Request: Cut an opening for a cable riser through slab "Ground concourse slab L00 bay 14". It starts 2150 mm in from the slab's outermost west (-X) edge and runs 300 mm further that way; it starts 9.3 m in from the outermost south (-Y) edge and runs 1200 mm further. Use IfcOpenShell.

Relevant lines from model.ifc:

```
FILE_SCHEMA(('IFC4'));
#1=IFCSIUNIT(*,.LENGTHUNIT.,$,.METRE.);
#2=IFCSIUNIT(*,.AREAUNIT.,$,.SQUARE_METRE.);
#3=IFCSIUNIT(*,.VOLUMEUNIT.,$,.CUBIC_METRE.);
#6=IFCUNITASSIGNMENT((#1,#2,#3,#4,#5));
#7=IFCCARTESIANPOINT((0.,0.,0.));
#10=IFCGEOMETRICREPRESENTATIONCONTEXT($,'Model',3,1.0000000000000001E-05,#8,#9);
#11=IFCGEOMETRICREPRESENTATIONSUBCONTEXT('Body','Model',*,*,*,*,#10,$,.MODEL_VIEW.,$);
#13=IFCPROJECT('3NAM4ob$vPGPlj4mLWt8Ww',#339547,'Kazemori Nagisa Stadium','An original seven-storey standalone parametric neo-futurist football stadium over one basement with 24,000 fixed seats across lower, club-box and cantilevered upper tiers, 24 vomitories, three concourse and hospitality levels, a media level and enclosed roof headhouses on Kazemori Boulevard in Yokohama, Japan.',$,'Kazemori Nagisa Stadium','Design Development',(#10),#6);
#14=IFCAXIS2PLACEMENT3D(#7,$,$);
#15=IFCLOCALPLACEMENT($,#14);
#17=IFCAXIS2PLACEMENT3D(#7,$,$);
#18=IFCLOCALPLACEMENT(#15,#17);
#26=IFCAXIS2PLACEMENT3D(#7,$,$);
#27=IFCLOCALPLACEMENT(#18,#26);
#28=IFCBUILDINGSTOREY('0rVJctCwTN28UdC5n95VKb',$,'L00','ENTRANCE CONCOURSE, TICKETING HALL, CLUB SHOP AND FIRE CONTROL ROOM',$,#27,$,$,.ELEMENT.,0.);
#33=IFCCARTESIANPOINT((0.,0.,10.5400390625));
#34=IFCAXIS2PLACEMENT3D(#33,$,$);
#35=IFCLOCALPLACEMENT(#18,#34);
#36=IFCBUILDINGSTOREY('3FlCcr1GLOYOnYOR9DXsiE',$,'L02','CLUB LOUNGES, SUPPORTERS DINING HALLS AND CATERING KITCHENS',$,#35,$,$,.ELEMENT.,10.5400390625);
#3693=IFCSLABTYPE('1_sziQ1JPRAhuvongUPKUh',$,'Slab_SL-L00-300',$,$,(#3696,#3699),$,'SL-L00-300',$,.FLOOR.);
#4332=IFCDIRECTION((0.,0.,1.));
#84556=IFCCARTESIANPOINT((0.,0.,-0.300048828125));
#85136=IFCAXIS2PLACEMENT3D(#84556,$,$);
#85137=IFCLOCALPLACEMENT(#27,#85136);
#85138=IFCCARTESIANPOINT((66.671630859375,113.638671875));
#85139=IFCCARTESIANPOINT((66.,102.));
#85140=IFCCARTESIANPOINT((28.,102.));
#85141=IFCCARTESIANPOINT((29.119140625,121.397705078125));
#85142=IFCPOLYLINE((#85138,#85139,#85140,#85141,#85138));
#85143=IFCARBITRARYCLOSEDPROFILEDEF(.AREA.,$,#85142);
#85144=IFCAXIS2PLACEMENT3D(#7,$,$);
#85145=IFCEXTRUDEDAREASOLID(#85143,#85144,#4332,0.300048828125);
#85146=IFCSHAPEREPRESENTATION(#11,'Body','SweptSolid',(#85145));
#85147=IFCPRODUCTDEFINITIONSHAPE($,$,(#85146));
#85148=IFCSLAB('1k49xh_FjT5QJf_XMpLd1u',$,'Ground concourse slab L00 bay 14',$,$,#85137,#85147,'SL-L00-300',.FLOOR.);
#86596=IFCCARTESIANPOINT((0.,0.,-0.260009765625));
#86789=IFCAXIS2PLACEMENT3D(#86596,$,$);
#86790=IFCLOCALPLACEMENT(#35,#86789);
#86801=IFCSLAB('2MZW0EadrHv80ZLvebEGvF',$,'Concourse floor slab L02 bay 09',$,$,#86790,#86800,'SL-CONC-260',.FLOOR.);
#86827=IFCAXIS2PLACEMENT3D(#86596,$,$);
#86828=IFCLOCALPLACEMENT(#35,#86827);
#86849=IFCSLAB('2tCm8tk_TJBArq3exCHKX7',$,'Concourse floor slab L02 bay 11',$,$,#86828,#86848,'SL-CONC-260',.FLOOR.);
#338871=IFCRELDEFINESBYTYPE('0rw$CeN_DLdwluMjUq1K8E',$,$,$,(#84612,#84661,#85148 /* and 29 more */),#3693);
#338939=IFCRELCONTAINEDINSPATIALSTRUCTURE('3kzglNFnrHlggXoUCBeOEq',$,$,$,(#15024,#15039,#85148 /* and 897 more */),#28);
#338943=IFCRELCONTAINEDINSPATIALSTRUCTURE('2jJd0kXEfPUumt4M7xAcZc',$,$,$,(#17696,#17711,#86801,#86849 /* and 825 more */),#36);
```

```python
import numpy as np
import ifcopenshell
import ifcopenshell.api.feature
import ifcopenshell.api.geometry
import ifcopenshell.api.root
import ifcopenshell.geom
import ifcopenshell.util.placement
import ifcopenshell.util.representation
import ifcopenshell.util.shape
import ifcopenshell.util.unit

model = ifcopenshell.open("model.ifc")
unit_scale = ifcopenshell.util.unit.calculate_unit_scale(model)
settings = ifcopenshell.geom.settings()


def volume(element):
    """Net volume in cubic metres, openings subtracted."""
    shape = ifcopenshell.geom.create_shape(settings, element)
    return ifcopenshell.util.shape.get_volume(shape.geometry)


slab = model.by_guid("1k49xh_FjT5QJf_XMpLd1u")
before = volume(slab)

# Extent in the slab's own axes, in metres. The edges named are its -X and -Y sides.
slab_shape = ifcopenshell.geom.create_shape(settings, slab)
vertices = ifcopenshell.util.shape.get_vertices(slab_shape.geometry)
x_min, y_min, bottom = vertices.min(axis=0)
top = vertices[:, 2].max()

opening = ifcopenshell.api.root.create_entity(model, ifc_class="IfcOpeningElement", name="Cable riser opening", predefined_type="OPENING")
context = ifcopenshell.util.representation.get_context(model, "Model", "Body", "MODEL_VIEW")
width, depth = 0.3, 1.2
outline = [(0.0, 0.0), (width, 0.0), (width, depth), (0.0, depth), (0.0, 0.0)]
# Overshoot both faces by 50 mm so the cut is clean.
shape = ifcopenshell.api.geometry.add_slab_representation(
    model, context=context, depth=top - bottom + 0.1, polyline=outline
)
ifcopenshell.api.geometry.assign_representation(model, product=opening, representation=shape)

matrix = ifcopenshell.util.placement.get_local_placement(slab.ObjectPlacement)
matrix[:, 3] = matrix @ np.append(np.array([x_min + 2.15, y_min + 9.3, bottom - 0.05]) / unit_scale, 1.0)
ifcopenshell.api.geometry.edit_object_placement(model, product=opening, matrix=matrix, is_si=False)
ifcopenshell.api.feature.add_feature(model, feature=opening, element=slab)

after = volume(slab)

print(f"slab volume {before:.3f} -> {after:.3f} m3")

model.write("model_edited.ifc")
```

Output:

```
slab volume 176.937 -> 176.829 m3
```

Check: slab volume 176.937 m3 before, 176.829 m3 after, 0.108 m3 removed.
